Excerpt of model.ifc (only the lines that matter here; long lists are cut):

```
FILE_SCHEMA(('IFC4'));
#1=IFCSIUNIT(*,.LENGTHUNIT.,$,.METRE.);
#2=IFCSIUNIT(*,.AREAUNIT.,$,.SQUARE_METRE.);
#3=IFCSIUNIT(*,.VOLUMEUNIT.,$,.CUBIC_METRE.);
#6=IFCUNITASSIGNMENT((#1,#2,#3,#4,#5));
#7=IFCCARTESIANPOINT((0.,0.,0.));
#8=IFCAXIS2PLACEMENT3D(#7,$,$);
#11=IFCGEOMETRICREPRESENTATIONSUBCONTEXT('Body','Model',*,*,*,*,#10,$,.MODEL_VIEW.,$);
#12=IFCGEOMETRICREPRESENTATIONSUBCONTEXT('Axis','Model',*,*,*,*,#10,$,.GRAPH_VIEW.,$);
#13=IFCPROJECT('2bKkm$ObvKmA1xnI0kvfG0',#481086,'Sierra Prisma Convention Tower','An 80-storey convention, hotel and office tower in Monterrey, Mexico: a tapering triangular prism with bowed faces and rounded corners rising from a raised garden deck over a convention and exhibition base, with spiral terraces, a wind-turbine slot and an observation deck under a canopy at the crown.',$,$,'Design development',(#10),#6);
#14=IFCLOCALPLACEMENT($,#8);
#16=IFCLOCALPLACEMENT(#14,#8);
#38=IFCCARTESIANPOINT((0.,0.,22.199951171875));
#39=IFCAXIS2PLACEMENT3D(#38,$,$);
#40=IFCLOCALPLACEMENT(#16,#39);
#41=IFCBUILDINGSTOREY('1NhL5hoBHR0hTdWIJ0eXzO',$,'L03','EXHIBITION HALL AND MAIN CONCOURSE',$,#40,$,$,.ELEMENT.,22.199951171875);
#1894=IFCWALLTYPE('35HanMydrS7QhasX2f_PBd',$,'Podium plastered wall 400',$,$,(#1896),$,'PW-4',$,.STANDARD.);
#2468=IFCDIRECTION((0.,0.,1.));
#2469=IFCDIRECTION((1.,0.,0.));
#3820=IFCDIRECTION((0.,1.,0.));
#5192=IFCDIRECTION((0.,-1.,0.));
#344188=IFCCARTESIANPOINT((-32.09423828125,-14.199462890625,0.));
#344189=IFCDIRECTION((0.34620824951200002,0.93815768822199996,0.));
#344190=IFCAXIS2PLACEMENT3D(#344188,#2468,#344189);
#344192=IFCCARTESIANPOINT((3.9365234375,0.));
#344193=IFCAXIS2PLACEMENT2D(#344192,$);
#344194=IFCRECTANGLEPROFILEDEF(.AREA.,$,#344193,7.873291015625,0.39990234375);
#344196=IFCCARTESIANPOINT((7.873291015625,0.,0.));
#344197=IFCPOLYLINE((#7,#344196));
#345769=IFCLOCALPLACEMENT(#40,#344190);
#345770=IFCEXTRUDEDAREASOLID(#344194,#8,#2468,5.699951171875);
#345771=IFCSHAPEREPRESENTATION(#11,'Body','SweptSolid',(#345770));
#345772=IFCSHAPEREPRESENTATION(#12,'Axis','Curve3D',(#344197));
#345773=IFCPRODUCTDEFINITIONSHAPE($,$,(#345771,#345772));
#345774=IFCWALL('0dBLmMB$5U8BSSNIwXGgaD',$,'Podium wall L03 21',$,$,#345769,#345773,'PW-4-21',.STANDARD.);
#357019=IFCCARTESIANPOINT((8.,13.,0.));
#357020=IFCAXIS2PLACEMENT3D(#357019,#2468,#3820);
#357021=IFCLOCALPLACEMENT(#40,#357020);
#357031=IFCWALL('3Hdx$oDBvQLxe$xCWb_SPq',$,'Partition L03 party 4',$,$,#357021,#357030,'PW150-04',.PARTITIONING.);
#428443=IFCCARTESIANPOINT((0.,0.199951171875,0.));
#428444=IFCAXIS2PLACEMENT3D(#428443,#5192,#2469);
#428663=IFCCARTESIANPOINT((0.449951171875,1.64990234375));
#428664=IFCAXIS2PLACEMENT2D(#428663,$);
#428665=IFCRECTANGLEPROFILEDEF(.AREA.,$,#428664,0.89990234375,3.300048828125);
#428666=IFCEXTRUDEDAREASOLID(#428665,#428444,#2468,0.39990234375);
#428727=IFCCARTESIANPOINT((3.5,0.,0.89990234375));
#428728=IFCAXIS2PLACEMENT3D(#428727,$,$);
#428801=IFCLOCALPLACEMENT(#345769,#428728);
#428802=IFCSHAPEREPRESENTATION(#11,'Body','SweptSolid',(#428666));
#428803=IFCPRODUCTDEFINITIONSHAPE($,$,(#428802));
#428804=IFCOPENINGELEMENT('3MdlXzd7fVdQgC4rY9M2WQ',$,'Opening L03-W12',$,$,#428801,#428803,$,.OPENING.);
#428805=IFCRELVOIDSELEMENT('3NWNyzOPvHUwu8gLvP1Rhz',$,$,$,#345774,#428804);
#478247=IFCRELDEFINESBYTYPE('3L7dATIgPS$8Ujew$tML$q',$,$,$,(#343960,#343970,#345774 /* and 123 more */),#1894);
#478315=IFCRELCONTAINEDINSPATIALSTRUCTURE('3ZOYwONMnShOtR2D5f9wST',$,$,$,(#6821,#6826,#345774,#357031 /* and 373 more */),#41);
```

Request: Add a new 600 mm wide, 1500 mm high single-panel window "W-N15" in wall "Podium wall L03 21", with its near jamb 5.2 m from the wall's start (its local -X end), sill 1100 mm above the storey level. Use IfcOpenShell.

```python
import numpy as np
import ifcopenshell
import ifcopenshell.api.feature
import ifcopenshell.api.geometry
import ifcopenshell.api.root
import ifcopenshell.api.spatial
import ifcopenshell.geom
import ifcopenshell.util.element
import ifcopenshell.util.placement
import ifcopenshell.util.representation
import ifcopenshell.util.shape
import ifcopenshell.util.unit

model = ifcopenshell.open("model.ifc")
unit_scale = ifcopenshell.util.unit.calculate_unit_scale(model)
settings = ifcopenshell.geom.settings()


def volume(element):
    """Net volume in cubic metres, openings subtracted."""
    shape = ifcopenshell.geom.create_shape(settings, element)
    return ifcopenshell.util.shape.get_volume(shape.geometry)


wall = model.by_id(345774)
storey = ifcopenshell.util.element.get_container(wall, ifc_class="IfcBuildingStorey")
context = ifcopenshell.util.representation.get_context(model, "Model", "Body", "MODEL_VIEW")
before = volume(wall)

width, height, from_end, sill = 0.6, 1.5, 5.2, 1.1  # metres

# The wall runs along its own X axis, and the end named is its -X end.
wall_shape = ifcopenshell.geom.create_shape(settings, wall)
x, y, z = ifcopenshell.util.shape.get_vertices(wall_shape.geometry).T
start = x.min() + from_end
face, thickness = float(y.min()), float(y.max() - y.min())
wall_matrix = ifcopenshell.util.placement.get_local_placement(wall.ObjectPlacement)
level = ifcopenshell.util.placement.get_local_placement(storey.ObjectPlacement)[2, 3]


def in_wall(x, y):
    """Placement at x, y metres in the wall's axes, at sill height."""
    matrix = wall_matrix.copy()
    matrix[:, 3] = wall_matrix @ np.array([x / unit_scale, y / unit_scale, 0.0, 1.0])
    matrix[2, 3] = level + sill / unit_scale
    return matrix


# Opening: a box that overshoots both wall faces by 50 mm.
opening = ifcopenshell.api.root.create_entity(model, ifc_class="IfcOpeningElement", predefined_type="OPENING")
box = ifcopenshell.api.geometry.add_wall_representation(
    model, context=context, length=width, height=height, thickness=thickness + 0.1
)
ifcopenshell.api.geometry.assign_representation(model, product=opening, representation=box)
ifcopenshell.api.geometry.edit_object_placement(model, product=opening, matrix=in_wall(start, face - 0.05), is_si=False)
ifcopenshell.api.feature.add_feature(model, feature=opening, element=wall)

window = ifcopenshell.api.root.create_entity(model, ifc_class="IfcWindow", name="W-N15", predefined_type="WINDOW")
window.OverallWidth, window.OverallHeight = width / unit_scale, height / unit_scale
window.PartitioningType = "SINGLE_PANEL"
body = ifcopenshell.api.geometry.add_window_representation(
    model,
    context=context,
    overall_width=window.OverallWidth,
    overall_height=window.OverallHeight,
    partition_type="SINGLE_PANEL",
)
ifcopenshell.api.geometry.assign_representation(model, product=window, representation=body)
ifcopenshell.api.spatial.assign_container(model, products=[window], relating_structure=storey)
ifcopenshell.api.feature.add_filling(model, opening=opening, element=window)

# Centre the window in the wall's thickness.
ifcopenshell.api.geometry.edit_object_placement(model, product=window, matrix=in_wall(start, face), is_si=False)
window_shape = ifcopenshell.geom.create_shape(settings, window)
depth = ifcopenshell.util.shape.get_vertices(window_shape.geometry)[:, 1]
offset = face + thickness / 2 - (depth.min() + depth.max()) / 2
ifcopenshell.api.geometry.edit_object_placement(model, product=window, matrix=in_wall(start, offset), is_si=False)

after = volume(wall)

print(f"wall volume {before:.3f} -> {after:.3f} m3")

model.write("model-out.ifc")
```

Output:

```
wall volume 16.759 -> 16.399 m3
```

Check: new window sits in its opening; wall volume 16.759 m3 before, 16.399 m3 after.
